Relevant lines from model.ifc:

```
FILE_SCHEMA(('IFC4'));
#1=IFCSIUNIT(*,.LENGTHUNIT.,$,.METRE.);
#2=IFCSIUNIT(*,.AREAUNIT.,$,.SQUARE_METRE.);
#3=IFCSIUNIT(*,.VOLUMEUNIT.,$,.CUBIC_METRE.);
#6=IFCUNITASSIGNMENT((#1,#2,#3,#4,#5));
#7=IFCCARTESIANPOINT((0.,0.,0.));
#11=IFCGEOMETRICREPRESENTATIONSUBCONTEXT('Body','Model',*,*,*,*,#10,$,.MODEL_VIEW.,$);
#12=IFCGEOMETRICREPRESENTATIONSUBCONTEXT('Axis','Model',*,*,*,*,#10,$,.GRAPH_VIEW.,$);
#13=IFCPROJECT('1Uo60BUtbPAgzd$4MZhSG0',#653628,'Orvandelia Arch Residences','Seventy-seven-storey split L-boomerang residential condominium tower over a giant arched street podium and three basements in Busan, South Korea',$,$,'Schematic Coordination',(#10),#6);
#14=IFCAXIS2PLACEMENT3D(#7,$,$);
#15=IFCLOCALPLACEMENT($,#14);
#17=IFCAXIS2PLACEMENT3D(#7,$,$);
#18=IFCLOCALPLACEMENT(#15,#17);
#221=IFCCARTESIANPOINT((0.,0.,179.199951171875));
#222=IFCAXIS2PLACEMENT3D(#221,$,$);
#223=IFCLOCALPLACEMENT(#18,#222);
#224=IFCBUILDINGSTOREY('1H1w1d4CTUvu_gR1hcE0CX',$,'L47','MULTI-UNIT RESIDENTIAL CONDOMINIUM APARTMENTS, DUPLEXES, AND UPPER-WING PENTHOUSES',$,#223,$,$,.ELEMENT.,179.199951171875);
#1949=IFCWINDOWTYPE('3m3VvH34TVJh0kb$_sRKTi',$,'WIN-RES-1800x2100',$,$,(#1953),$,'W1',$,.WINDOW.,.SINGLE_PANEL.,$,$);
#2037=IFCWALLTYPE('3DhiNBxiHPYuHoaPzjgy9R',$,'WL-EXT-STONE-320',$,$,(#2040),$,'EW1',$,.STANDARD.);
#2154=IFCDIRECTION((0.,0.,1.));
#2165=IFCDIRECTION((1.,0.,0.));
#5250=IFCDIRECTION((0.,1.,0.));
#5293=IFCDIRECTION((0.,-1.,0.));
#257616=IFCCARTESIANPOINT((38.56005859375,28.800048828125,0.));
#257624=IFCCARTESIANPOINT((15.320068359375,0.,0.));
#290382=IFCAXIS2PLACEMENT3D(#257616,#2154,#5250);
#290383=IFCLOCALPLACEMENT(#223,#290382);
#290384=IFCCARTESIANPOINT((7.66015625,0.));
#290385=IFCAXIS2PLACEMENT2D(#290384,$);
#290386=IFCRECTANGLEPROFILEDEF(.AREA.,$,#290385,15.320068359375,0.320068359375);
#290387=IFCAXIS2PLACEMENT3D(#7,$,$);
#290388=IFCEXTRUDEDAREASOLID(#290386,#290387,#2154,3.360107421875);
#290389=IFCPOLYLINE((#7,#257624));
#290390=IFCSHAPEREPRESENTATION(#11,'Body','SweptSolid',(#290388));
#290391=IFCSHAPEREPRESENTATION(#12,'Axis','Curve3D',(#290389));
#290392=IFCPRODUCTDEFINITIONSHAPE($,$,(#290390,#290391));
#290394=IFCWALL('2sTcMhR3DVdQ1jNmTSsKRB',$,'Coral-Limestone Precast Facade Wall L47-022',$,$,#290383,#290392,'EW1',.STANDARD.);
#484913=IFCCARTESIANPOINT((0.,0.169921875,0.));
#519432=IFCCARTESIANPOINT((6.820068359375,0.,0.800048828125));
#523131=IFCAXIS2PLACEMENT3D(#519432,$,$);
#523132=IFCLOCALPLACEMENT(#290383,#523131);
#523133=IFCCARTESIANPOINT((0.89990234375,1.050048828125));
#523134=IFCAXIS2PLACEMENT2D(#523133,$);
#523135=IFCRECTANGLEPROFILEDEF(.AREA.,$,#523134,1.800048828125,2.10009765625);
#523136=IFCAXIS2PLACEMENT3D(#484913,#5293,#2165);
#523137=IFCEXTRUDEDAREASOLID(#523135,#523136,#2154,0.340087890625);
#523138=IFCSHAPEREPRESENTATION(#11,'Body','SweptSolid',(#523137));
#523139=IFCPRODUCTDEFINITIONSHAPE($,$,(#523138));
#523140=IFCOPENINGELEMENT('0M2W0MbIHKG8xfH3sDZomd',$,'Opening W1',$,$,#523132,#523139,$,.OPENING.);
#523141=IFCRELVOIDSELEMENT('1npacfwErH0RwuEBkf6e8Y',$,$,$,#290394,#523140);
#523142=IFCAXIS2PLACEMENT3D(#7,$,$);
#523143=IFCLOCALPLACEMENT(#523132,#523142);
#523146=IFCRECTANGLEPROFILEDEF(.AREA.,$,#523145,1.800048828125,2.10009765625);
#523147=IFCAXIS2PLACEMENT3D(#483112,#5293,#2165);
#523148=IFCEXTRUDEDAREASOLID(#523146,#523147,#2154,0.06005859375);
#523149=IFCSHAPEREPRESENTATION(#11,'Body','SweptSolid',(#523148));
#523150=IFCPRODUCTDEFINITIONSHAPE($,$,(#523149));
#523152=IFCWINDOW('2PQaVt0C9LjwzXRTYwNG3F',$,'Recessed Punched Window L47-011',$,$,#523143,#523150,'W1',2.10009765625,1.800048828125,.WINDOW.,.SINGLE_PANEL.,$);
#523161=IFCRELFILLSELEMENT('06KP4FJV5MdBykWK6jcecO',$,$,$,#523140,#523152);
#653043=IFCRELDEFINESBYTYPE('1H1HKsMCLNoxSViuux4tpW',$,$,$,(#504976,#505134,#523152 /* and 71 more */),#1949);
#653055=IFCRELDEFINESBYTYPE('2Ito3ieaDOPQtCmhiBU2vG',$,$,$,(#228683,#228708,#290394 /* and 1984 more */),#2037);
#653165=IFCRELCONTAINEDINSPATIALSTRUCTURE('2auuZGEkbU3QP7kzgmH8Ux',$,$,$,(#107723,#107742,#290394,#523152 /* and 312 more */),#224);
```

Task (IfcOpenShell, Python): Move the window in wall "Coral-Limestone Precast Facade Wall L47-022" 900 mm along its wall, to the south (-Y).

```python
import ifcopenshell
import ifcopenshell.api.geometry
import ifcopenshell.util.placement

model = ifcopenshell.open("model.ifc")

window = model.by_guid("2PQaVt0C9LjwzXRTYwNG3F")
opening = window.FillsVoids[0].RelatingOpeningElement
wall = opening.VoidsElements[0].RelatingBuildingElement

wall_matrix = ifcopenshell.util.placement.get_local_placement(wall.ObjectPlacement)
shift = wall_matrix[:3, 0] * -0.9
before = ifcopenshell.util.placement.get_local_placement(window.ObjectPlacement)[:3, 3].copy()

# The window is placed relative to its opening, so it follows when the opening moves.
matrix = ifcopenshell.util.placement.get_local_placement(opening.ObjectPlacement)
matrix[:3, 3] += shift
ifcopenshell.api.geometry.edit_object_placement(
    model, product=opening, matrix=matrix, is_si=False, should_transform_children=True
)

after = ifcopenshell.util.placement.get_local_placement(window.ObjectPlacement)[:3, 3]
print("window moved by", (after - before).round(3) + 0.0)

model.write("model_edited.ifc")
```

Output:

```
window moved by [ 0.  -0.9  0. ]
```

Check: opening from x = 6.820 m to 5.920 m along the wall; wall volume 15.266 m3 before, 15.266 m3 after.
